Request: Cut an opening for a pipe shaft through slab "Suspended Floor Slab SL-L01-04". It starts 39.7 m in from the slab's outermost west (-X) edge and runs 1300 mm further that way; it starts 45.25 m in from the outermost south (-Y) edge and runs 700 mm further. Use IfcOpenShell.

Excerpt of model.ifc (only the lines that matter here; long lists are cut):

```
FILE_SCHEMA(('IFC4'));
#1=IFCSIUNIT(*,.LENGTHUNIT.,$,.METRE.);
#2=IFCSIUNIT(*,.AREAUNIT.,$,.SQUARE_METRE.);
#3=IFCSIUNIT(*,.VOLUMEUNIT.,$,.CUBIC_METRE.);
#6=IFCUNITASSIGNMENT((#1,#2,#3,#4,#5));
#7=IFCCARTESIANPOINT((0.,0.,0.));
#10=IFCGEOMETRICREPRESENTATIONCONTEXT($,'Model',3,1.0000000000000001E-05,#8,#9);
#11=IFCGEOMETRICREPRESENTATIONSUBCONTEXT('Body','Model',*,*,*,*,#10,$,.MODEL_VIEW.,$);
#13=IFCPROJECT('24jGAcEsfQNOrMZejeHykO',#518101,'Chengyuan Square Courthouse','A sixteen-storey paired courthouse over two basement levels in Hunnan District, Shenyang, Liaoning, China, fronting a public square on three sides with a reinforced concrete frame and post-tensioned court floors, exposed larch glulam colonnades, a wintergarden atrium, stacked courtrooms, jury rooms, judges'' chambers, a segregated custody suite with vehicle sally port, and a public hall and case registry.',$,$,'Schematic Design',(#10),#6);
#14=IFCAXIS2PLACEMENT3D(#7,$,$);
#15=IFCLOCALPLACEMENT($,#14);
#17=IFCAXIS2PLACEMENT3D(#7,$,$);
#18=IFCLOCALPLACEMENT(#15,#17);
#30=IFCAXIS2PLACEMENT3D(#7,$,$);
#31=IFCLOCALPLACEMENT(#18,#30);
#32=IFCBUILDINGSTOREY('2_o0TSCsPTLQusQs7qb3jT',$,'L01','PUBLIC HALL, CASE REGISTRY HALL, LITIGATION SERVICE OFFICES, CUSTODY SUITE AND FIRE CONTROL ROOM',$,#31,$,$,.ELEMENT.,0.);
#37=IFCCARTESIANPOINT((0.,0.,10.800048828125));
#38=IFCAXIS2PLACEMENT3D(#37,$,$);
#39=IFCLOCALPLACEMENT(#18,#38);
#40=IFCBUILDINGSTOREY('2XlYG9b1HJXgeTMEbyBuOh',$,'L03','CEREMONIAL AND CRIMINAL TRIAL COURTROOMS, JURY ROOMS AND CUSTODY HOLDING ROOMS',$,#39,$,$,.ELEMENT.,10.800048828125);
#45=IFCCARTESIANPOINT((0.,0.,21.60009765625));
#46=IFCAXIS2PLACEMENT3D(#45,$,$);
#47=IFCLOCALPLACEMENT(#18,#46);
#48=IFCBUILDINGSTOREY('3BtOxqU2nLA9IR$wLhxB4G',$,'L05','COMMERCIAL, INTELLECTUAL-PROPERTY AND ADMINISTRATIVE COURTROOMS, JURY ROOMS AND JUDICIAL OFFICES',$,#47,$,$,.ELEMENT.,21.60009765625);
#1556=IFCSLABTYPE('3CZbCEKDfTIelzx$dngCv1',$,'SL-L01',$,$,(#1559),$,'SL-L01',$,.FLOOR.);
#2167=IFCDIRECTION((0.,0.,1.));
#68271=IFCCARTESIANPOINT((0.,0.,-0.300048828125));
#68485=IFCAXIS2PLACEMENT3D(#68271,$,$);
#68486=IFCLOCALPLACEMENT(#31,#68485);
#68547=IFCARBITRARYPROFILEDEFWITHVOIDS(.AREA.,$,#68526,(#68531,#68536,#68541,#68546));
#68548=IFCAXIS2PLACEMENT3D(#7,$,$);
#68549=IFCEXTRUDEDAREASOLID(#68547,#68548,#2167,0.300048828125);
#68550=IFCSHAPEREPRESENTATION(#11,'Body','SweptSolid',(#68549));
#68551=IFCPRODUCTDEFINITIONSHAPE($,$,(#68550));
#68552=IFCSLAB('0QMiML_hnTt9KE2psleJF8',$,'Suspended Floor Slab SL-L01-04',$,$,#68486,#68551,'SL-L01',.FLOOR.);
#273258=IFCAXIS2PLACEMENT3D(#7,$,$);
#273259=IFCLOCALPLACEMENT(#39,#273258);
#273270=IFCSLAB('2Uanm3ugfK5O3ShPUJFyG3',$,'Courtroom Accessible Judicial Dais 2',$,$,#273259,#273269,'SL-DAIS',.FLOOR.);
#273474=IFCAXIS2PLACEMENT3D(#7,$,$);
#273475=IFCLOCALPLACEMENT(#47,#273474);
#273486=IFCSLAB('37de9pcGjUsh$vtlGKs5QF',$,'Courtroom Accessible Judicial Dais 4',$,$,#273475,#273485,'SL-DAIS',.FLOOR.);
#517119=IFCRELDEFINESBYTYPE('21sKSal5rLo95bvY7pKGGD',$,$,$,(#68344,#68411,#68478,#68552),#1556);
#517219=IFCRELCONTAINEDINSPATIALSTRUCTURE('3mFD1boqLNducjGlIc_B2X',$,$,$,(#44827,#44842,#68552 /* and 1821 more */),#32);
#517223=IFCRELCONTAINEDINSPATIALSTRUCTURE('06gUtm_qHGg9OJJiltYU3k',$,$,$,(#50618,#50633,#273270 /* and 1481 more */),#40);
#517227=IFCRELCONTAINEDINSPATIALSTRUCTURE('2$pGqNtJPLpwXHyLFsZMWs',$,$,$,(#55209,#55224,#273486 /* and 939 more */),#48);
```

```python
import numpy as np
import ifcopenshell
import ifcopenshell.api.feature
import ifcopenshell.api.geometry
import ifcopenshell.api.root
import ifcopenshell.geom
import ifcopenshell.util.placement
import ifcopenshell.util.representation
import ifcopenshell.util.shape
import ifcopenshell.util.unit

model = ifcopenshell.open("model.ifc")
unit_scale = ifcopenshell.util.unit.calculate_unit_scale(model)
settings = ifcopenshell.geom.settings()


def volume(element):
    """Net volume in cubic metres, openings subtracted."""
    shape = ifcopenshell.geom.create_shape(settings, element)
    return ifcopenshell.util.shape.get_volume(shape.geometry)


slab = model.by_guid("0QMiML_hnTt9KE2psleJF8")
before = volume(slab)

# Extent in the slab's own axes, in metres. The edges named are its -X and -Y sides.
slab_shape = ifcopenshell.geom.create_shape(settings, slab)
vertices = ifcopenshell.util.shape.get_vertices(slab_shape.geometry)
x_min, y_min, bottom = vertices.min(axis=0)
top = vertices[:, 2].max()

opening = ifcopenshell.api.root.create_entity(model, ifc_class="IfcOpeningElement", name="Pipe shaft opening", predefined_type="OPENING")
context = ifcopenshell.util.representation.get_context(model, "Model", "Body", "MODEL_VIEW")
width, depth = 1.3, 0.7
outline = [(0.0, 0.0), (width, 0.0), (width, depth), (0.0, depth), (0.0, 0.0)]
# Overshoot both faces by 50 mm so the cut is clean.
shape = ifcopenshell.api.geometry.add_slab_representation(
    model, context=context, depth=top - bottom + 0.1, polyline=outline
)
ifcopenshell.api.geometry.assign_representation(model, product=opening, representation=shape)

matrix = ifcopenshell.util.placement.get_local_placement(slab.ObjectPlacement)
matrix[:, 3] = matrix @ np.append(np.array([x_min + 39.7, y_min + 45.25, bottom - 0.05]) / unit_scale, 1.0)
ifcopenshell.api.geometry.edit_object_placement(model, product=opening, matrix=matrix, is_si=False)
ifcopenshell.api.feature.add_feature(model, feature=opening, element=slab)

after = volume(slab)

print(f"slab volume {before:.3f} -> {after:.3f} m3")

model.write("model_updated.ifc")
```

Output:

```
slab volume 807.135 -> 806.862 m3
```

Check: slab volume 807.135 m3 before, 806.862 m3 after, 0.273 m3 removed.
